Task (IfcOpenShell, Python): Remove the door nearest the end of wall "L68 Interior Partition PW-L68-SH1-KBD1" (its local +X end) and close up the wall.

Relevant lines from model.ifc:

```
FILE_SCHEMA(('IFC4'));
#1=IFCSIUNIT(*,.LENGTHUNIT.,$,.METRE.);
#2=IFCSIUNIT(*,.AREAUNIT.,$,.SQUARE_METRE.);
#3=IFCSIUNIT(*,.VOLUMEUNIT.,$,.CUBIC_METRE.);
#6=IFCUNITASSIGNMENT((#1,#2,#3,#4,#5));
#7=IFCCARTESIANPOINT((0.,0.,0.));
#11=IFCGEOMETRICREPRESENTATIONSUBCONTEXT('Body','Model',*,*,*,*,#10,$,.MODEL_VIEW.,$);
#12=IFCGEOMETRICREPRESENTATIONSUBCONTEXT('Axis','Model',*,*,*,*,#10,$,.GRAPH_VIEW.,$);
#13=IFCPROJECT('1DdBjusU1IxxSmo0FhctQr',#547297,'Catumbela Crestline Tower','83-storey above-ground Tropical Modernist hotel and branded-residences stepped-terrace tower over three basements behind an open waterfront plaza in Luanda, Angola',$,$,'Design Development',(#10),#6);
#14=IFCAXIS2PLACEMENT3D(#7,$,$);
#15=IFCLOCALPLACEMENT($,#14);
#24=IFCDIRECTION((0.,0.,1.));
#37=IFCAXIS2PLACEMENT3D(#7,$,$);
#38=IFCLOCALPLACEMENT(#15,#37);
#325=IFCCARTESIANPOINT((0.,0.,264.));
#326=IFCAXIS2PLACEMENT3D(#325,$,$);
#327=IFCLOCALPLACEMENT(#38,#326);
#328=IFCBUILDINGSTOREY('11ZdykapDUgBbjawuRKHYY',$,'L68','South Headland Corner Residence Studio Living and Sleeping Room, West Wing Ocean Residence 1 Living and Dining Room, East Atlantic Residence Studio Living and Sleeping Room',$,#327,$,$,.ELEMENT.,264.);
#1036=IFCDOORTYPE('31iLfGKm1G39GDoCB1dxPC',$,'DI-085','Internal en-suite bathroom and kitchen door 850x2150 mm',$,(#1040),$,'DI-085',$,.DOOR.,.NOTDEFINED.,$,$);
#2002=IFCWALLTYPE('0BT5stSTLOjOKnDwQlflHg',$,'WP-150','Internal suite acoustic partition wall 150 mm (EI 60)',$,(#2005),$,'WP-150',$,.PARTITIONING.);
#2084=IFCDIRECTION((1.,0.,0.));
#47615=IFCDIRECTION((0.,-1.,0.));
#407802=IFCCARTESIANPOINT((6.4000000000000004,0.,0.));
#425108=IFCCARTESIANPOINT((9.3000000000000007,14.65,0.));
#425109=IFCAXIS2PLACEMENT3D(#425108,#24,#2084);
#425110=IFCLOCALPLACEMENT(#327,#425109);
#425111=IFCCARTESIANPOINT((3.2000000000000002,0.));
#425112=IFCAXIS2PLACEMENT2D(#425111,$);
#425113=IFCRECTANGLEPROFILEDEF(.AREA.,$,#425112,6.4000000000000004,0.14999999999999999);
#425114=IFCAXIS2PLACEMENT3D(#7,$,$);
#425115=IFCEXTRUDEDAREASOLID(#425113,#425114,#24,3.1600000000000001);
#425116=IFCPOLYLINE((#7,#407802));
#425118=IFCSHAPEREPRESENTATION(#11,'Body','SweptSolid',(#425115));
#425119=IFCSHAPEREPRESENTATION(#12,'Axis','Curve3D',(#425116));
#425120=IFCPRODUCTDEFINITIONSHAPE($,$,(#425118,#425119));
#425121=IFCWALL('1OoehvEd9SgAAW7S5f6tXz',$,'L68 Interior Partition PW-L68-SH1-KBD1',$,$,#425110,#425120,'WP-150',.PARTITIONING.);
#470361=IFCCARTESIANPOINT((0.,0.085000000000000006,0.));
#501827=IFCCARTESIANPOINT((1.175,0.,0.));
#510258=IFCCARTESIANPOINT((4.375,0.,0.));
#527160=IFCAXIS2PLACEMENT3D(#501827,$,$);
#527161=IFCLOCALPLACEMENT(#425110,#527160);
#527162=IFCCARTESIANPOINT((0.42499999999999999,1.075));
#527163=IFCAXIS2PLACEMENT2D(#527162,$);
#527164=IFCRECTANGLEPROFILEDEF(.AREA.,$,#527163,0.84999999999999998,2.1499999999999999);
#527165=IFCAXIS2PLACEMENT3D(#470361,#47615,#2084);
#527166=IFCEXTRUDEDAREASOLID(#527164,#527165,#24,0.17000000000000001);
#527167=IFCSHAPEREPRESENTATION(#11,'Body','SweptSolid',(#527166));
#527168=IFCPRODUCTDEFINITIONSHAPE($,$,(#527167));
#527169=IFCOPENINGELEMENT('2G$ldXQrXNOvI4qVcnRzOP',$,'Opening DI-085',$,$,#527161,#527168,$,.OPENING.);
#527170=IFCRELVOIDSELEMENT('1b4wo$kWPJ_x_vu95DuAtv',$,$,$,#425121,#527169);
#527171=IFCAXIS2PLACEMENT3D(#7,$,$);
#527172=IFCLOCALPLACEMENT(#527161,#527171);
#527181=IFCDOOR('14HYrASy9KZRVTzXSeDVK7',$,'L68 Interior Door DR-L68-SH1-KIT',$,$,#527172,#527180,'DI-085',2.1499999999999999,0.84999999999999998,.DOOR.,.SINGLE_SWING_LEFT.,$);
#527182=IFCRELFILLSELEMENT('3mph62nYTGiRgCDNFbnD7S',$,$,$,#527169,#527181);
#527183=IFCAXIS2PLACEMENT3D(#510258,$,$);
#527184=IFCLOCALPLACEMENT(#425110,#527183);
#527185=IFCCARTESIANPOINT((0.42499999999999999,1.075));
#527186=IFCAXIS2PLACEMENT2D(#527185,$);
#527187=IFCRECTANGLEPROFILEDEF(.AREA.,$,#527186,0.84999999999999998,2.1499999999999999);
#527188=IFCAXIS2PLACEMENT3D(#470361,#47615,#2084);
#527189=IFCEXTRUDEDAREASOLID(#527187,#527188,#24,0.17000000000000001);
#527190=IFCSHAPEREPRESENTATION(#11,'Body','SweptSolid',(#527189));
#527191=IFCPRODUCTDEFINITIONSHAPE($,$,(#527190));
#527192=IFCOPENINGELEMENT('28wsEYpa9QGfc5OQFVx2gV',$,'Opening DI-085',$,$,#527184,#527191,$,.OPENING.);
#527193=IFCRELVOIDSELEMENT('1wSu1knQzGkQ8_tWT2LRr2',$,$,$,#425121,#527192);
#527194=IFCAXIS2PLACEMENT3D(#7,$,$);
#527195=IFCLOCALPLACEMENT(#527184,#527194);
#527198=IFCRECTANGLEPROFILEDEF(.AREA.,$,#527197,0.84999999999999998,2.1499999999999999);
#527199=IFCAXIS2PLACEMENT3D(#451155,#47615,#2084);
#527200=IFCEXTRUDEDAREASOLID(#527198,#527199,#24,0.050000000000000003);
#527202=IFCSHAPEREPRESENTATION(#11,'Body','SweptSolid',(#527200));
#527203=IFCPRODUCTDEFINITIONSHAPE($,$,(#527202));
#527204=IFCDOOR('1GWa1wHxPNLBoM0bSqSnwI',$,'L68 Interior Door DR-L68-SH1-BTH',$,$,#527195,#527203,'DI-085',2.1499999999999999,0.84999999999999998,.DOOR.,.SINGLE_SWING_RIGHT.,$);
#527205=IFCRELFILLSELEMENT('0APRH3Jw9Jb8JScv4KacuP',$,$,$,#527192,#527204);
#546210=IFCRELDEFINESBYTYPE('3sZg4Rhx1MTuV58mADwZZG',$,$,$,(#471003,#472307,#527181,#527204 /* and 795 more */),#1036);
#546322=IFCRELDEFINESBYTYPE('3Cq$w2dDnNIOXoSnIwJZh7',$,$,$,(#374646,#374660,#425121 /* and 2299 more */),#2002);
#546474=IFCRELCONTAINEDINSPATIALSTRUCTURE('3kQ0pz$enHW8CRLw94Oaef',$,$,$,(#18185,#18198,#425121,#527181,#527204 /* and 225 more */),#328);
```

```python
import ifcopenshell
import ifcopenshell.api.feature
import ifcopenshell.api.root
import ifcopenshell.geom
import ifcopenshell.util.shape

model = ifcopenshell.open("model.ifc")
settings = ifcopenshell.geom.settings()


def volume(element):
    """Net volume in cubic metres, openings subtracted."""
    shape = ifcopenshell.geom.create_shape(settings, element)
    return ifcopenshell.util.shape.get_volume(shape.geometry)


door = model.by_id(527204)
opening = door.FillsVoids[0].RelatingOpeningElement
wall = opening.VoidsElements[0].RelatingBuildingElement
before = volume(wall)

ifcopenshell.api.root.remove_product(model, product=door)
ifcopenshell.api.feature.remove_feature(model, feature=opening)

after = volume(wall)

print(f"wall volume {before:.3f} -> {after:.3f} m3")

model.write("model-out.ifc")
```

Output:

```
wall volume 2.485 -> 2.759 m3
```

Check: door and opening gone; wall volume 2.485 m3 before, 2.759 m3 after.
